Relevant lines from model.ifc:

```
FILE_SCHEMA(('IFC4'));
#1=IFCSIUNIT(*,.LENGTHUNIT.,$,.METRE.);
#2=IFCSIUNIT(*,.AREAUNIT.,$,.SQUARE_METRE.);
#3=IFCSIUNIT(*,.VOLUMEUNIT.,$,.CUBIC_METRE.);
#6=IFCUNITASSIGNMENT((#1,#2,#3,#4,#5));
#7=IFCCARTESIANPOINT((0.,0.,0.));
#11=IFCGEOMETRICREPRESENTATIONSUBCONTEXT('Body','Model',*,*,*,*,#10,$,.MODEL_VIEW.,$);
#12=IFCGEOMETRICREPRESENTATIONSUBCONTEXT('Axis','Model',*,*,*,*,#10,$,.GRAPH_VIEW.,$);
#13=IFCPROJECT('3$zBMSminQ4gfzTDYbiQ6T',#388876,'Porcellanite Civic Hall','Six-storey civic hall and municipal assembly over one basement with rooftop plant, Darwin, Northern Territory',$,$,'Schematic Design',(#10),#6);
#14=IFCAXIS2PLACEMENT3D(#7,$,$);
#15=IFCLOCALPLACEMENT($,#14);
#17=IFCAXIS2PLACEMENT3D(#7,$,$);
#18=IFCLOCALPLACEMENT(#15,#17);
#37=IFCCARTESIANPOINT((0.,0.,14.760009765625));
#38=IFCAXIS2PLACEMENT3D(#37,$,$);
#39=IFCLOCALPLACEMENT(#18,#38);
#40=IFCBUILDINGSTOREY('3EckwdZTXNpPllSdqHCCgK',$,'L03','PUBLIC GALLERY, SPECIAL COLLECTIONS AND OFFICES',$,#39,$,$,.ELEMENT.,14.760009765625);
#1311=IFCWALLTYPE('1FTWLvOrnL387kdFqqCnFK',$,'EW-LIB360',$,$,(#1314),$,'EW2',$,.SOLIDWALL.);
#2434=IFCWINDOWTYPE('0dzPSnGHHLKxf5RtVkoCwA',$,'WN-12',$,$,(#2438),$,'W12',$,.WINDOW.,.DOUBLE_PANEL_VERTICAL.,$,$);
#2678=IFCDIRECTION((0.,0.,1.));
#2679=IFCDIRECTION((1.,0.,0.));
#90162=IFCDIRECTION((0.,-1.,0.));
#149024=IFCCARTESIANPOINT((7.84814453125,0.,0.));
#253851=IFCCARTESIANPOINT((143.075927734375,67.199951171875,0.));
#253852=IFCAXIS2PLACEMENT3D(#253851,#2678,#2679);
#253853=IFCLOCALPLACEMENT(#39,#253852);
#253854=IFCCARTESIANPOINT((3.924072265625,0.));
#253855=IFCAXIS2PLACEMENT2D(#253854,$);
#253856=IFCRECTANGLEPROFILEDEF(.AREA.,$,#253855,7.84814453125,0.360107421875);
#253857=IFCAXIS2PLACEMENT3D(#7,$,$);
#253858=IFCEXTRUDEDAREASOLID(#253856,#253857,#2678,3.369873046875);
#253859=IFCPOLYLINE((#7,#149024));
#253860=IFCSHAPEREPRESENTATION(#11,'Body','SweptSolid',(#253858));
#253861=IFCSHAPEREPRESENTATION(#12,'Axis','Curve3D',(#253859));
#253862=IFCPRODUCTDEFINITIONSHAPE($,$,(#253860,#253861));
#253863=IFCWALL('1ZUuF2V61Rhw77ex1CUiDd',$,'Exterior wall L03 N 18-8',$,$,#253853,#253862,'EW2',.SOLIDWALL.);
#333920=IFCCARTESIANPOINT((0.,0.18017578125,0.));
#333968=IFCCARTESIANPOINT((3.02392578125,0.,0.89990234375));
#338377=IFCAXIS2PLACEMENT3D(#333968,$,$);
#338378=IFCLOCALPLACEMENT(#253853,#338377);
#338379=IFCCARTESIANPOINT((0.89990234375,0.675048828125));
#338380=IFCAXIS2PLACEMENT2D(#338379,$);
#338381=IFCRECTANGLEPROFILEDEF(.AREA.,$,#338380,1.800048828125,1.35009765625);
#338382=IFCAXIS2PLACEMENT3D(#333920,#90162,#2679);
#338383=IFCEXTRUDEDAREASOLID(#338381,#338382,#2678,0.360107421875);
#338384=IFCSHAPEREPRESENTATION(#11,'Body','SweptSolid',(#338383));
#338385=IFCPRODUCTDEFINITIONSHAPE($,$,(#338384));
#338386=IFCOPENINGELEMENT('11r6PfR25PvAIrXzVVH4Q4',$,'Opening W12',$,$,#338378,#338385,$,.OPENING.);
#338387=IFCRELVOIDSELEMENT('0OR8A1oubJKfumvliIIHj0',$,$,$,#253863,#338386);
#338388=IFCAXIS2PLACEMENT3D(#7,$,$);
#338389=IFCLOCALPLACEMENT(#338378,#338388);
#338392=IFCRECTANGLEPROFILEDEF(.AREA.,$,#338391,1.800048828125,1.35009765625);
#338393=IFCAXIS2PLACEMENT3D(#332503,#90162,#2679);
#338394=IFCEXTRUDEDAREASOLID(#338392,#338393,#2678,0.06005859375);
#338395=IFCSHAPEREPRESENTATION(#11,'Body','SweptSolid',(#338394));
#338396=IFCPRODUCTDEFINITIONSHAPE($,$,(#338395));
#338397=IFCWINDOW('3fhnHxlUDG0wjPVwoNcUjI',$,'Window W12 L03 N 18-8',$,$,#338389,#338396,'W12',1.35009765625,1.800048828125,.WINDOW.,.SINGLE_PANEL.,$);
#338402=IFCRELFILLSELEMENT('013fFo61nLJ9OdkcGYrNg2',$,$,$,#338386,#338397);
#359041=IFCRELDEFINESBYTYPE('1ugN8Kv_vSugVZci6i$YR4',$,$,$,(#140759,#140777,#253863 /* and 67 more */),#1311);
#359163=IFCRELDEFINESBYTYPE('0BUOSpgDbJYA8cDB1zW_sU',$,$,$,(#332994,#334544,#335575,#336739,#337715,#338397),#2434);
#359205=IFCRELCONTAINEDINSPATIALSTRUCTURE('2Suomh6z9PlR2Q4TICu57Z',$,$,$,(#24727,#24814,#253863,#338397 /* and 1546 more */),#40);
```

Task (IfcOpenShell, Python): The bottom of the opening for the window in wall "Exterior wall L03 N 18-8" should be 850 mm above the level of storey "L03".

```python
import numpy as np
import ifcopenshell
import ifcopenshell.api.geometry
import ifcopenshell.geom
import ifcopenshell.util.element
import ifcopenshell.util.placement
import ifcopenshell.util.shape
import ifcopenshell.util.unit

model = ifcopenshell.open("model.ifc")
unit_scale = ifcopenshell.util.unit.calculate_unit_scale(model)

window = model.by_guid("3fhnHxlUDG0wjPVwoNcUjI")
opening = window.FillsVoids[0].RelatingOpeningElement
storey = ifcopenshell.util.element.get_container(window, ifc_class="IfcBuildingStorey")
level = ifcopenshell.util.placement.get_local_placement(storey.ObjectPlacement)[2, 3]

# The opening's origin need not be at the sill, so measure its lowest point.
shape = ifcopenshell.geom.create_shape(ifcopenshell.geom.settings(), opening)
bottom = ifcopenshell.util.shape.get_shape_bottom_elevation(shape, shape.geometry) / unit_scale
dz = level + 0.85 - bottom

shift = np.array([0.0, 0.0, dz])
# The window is placed relative to its opening, so it follows when the opening moves.
matrix = ifcopenshell.util.placement.get_local_placement(opening.ObjectPlacement)
matrix[:3, 3] += shift
ifcopenshell.api.geometry.edit_object_placement(
    model, product=opening, matrix=matrix, is_si=False, should_transform_children=True
)

print(f"moved by {dz * unit_scale:+.3f} m")

model.write("model_rev.ifc")
```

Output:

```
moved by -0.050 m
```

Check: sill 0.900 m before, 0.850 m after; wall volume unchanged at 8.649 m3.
